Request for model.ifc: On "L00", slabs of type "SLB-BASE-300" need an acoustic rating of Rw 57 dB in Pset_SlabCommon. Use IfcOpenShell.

First a look at what the model holds.

```python
import ifcopenshell
import ifcopenshell.util.element

model = ifcopenshell.open("model.ifc")
print(model.schema)
storey = next(s for s in model.by_type("IfcBuildingStorey") if s.Name == "L00")
slabs = [e for e in ifcopenshell.util.element.get_decomposition(storey) if e.is_a("IfcSlab")]
seen = {}
for e in slabs:
    element_type = ifcopenshell.util.element.get_type(e)
    key = (element_type.Name if element_type != e and element_type else None, ifcopenshell.util.element.get_pset(e, "Pset_SlabCommon", "AcousticRating"))
    seen[key] = seen.get(key, 0) + 1
for (name, value), count in sorted(seen.items(), key=str):
    print(count, "x", name, "|", value)
```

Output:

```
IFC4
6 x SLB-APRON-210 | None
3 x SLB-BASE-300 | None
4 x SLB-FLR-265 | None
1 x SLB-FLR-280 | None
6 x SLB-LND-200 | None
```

```python
import ifcopenshell
import ifcopenshell.api.pset
import ifcopenshell.util.element

model = ifcopenshell.open("model.ifc")

storey = next(s for s in model.by_type("IfcBuildingStorey") if s.Name == "L00")
slabs = [e for e in ifcopenshell.util.element.get_decomposition(storey) if e.is_a("IfcSlab")]

count = 0
for e in slabs:
    element_type = ifcopenshell.util.element.get_type(e)
    if element_type in (None, e) or element_type.Name != "SLB-BASE-300":
        continue
    # add_pset returns the element's existing set when there is one.
    pset = ifcopenshell.api.pset.add_pset(model, product=e, name="Pset_SlabCommon")
    ifcopenshell.api.pset.edit_pset(model, pset=pset, properties={"AcousticRating": "Rw 57 dB"})
    count += 1

print(count, "slabs updated")

model.write("model_updated.ifc")
```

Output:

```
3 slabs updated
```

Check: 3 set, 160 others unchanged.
